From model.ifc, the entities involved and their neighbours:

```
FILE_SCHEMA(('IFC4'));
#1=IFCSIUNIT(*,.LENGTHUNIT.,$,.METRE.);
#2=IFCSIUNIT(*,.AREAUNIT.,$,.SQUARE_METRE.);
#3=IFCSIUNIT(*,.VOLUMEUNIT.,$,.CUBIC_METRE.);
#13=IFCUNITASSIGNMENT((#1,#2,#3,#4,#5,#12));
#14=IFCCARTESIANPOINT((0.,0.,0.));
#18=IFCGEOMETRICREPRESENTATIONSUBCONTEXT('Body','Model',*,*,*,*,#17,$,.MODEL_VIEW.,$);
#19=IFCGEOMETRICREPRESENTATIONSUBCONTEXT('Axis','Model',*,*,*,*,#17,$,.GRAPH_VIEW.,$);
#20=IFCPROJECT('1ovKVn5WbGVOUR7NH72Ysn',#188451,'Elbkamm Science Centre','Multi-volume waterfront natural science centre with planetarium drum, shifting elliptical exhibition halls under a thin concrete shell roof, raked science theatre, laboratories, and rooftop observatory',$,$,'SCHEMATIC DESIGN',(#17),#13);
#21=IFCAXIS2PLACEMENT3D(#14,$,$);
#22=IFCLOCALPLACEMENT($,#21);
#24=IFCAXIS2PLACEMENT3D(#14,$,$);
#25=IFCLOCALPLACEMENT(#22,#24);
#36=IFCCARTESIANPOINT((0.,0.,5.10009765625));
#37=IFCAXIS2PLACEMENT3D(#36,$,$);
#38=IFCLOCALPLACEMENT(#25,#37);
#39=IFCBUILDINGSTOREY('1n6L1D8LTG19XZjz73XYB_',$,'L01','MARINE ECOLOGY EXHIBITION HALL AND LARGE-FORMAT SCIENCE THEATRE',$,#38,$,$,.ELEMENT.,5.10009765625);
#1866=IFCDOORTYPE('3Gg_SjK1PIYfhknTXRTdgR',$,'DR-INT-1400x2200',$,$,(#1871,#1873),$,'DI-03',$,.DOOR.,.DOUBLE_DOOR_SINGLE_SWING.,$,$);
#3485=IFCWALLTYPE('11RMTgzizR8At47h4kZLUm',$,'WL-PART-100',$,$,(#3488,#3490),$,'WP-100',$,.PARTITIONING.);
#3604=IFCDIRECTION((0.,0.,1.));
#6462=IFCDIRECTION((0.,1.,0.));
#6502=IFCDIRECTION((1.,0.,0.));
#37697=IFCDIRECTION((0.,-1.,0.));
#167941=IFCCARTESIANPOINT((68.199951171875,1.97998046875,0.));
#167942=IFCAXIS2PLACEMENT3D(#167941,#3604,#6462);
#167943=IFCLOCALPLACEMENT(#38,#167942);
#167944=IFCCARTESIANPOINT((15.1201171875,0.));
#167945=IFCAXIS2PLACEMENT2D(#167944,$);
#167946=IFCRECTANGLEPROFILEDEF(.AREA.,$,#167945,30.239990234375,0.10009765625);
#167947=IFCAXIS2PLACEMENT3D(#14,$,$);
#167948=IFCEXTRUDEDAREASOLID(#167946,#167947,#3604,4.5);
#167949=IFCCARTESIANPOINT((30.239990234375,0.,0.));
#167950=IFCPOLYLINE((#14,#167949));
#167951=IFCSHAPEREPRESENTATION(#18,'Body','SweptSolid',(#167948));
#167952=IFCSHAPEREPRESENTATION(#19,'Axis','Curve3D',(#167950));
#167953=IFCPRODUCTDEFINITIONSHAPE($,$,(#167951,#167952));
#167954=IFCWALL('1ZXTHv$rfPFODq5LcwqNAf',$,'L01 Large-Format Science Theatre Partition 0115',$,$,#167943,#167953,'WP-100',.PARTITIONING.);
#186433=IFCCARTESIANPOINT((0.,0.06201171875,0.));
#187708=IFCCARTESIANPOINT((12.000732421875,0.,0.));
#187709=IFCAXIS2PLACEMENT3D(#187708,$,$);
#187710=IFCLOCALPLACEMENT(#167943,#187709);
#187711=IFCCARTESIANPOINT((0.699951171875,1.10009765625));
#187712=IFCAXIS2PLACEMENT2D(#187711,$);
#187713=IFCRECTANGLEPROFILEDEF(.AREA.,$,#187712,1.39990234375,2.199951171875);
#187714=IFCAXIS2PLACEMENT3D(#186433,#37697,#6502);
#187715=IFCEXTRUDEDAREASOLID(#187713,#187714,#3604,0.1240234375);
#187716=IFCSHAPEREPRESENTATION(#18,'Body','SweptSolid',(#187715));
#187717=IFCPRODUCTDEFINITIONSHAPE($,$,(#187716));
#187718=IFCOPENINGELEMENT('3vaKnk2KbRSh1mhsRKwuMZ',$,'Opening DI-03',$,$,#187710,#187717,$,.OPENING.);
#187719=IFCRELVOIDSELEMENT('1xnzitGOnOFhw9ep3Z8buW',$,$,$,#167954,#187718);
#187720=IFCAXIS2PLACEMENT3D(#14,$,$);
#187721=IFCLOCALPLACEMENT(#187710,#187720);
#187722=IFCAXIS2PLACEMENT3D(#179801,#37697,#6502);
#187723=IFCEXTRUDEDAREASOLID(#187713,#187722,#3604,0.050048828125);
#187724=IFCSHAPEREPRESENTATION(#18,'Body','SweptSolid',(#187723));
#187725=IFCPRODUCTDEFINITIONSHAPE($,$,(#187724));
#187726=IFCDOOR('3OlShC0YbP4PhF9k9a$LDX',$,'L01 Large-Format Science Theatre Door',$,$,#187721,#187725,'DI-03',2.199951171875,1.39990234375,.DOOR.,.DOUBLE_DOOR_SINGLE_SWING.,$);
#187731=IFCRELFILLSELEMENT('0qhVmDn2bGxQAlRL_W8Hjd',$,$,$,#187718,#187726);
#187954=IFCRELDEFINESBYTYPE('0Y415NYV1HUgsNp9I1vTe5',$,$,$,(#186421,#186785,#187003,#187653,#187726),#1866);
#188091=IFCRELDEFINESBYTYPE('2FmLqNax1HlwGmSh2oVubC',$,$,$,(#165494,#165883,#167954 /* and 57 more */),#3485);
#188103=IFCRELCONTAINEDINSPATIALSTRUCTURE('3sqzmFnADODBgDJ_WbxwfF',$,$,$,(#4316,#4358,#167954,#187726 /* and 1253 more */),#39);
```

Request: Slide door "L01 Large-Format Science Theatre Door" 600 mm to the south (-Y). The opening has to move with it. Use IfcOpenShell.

```python
import ifcopenshell
import ifcopenshell.api.geometry
import ifcopenshell.util.placement

model = ifcopenshell.open("model.ifc")

door = model.by_guid("3OlShC0YbP4PhF9k9a$LDX")
opening = door.FillsVoids[0].RelatingOpeningElement
wall = opening.VoidsElements[0].RelatingBuildingElement

wall_matrix = ifcopenshell.util.placement.get_local_placement(wall.ObjectPlacement)
shift = wall_matrix[:3, 0] * -0.6
before = ifcopenshell.util.placement.get_local_placement(door.ObjectPlacement)[:3, 3].copy()

# The door is placed relative to its opening, so it follows when the opening moves.
matrix = ifcopenshell.util.placement.get_local_placement(opening.ObjectPlacement)
matrix[:3, 3] += shift
ifcopenshell.api.geometry.edit_object_placement(
    model, product=opening, matrix=matrix, is_si=False, should_transform_children=True
)

after = ifcopenshell.util.placement.get_local_placement(door.ObjectPlacement)[:3, 3]
print("door moved by", (after - before).round(3) + 0.0)

model.write("model_edited.ifc")
```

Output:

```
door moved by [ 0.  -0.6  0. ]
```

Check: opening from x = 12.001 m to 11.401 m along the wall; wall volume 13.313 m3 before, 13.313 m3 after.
